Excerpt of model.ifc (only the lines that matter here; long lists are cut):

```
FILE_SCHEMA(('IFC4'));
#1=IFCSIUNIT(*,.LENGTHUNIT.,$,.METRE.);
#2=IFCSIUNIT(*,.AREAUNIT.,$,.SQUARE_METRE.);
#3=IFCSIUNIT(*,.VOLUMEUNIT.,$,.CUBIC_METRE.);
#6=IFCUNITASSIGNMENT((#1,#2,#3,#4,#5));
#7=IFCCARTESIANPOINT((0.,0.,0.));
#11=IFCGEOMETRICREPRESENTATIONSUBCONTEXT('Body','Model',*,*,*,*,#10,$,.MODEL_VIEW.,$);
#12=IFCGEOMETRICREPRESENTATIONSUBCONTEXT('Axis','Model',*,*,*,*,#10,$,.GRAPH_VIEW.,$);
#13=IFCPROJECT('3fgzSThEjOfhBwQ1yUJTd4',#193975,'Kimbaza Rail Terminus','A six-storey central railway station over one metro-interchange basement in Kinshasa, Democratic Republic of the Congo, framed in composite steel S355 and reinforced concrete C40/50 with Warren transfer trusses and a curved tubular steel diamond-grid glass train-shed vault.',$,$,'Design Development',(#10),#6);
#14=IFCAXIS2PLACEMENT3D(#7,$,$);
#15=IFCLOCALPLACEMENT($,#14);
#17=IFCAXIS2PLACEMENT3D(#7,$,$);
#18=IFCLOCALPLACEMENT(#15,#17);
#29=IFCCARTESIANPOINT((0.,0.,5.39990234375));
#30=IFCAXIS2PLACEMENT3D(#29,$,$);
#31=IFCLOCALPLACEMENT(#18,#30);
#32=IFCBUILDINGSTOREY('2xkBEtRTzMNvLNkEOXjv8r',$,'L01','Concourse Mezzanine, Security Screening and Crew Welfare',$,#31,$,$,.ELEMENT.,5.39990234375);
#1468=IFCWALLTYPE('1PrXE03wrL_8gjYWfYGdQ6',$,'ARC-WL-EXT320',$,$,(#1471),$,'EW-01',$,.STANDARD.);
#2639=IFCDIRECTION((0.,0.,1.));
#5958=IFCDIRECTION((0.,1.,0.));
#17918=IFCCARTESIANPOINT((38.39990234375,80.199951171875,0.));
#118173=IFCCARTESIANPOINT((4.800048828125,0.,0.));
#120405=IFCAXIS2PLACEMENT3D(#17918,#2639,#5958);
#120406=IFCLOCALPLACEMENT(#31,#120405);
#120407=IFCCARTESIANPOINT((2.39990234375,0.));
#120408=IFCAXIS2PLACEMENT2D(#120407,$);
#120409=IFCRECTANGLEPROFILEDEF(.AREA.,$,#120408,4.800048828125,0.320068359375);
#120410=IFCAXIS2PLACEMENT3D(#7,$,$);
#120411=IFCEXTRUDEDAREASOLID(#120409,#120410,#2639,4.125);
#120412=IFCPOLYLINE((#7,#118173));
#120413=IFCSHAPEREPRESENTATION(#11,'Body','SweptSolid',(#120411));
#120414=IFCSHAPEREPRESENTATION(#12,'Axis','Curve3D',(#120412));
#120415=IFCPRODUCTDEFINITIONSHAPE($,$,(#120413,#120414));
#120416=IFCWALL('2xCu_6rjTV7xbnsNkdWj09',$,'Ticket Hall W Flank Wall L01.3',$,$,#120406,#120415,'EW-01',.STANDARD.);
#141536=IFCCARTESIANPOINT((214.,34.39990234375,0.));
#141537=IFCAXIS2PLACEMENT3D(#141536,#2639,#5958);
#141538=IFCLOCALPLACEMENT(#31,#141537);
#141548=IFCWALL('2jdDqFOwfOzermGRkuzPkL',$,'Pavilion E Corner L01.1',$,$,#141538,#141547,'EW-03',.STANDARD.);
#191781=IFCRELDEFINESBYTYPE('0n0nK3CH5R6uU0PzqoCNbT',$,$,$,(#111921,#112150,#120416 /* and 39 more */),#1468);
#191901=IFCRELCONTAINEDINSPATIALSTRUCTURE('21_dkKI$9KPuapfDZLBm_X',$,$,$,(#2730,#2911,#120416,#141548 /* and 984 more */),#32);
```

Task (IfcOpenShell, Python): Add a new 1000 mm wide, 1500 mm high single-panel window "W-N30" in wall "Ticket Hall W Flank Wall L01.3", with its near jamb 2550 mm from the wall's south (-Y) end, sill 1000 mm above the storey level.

```python
import numpy as np
import ifcopenshell
import ifcopenshell.api.feature
import ifcopenshell.api.geometry
import ifcopenshell.api.root
import ifcopenshell.api.spatial
import ifcopenshell.geom
import ifcopenshell.util.element
import ifcopenshell.util.placement
import ifcopenshell.util.representation
import ifcopenshell.util.shape
import ifcopenshell.util.unit

model = ifcopenshell.open("model.ifc")
unit_scale = ifcopenshell.util.unit.calculate_unit_scale(model)
settings = ifcopenshell.geom.settings()


def volume(element):
    """Net volume in cubic metres, openings subtracted."""
    shape = ifcopenshell.geom.create_shape(settings, element)
    return ifcopenshell.util.shape.get_volume(shape.geometry)


wall = model.by_id(120416)
storey = ifcopenshell.util.element.get_container(wall, ifc_class="IfcBuildingStorey")
context = ifcopenshell.util.representation.get_context(model, "Model", "Body", "MODEL_VIEW")
before = volume(wall)

width, height, from_end, sill = 1, 1.5, 2.55, 1  # metres

# The wall runs along its own X axis, and the end named is its -X end.
wall_shape = ifcopenshell.geom.create_shape(settings, wall)
x, y, z = ifcopenshell.util.shape.get_vertices(wall_shape.geometry).T
start = x.min() + from_end
face, thickness = float(y.min()), float(y.max() - y.min())
wall_matrix = ifcopenshell.util.placement.get_local_placement(wall.ObjectPlacement)
level = ifcopenshell.util.placement.get_local_placement(storey.ObjectPlacement)[2, 3]


def in_wall(x, y):
    """Placement at x, y metres in the wall's axes, at sill height."""
    matrix = wall_matrix.copy()
    matrix[:, 3] = wall_matrix @ np.array([x / unit_scale, y / unit_scale, 0.0, 1.0])
    matrix[2, 3] = level + sill / unit_scale
    return matrix


# Opening: a box that overshoots both wall faces by 50 mm.
opening = ifcopenshell.api.root.create_entity(model, ifc_class="IfcOpeningElement", predefined_type="OPENING")
box = ifcopenshell.api.geometry.add_wall_representation(
    model, context=context, length=width, height=height, thickness=thickness + 0.1
)
ifcopenshell.api.geometry.assign_representation(model, product=opening, representation=box)
ifcopenshell.api.geometry.edit_object_placement(model, product=opening, matrix=in_wall(start, face - 0.05), is_si=False)
ifcopenshell.api.feature.add_feature(model, feature=opening, element=wall)

window = ifcopenshell.api.root.create_entity(model, ifc_class="IfcWindow", name="W-N30", predefined_type="WINDOW")
window.OverallWidth, window.OverallHeight = width / unit_scale, height / unit_scale
window.PartitioningType = "SINGLE_PANEL"
body = ifcopenshell.api.geometry.add_window_representation(
    model,
    context=context,
    overall_width=window.OverallWidth,
    overall_height=window.OverallHeight,
    partition_type="SINGLE_PANEL",
)
ifcopenshell.api.geometry.assign_representation(model, product=window, representation=body)
ifcopenshell.api.spatial.assign_container(model, products=[window], relating_structure=storey)
ifcopenshell.api.feature.add_filling(model, opening=opening, element=window)

# Centre the window in the wall's thickness.
ifcopenshell.api.geometry.edit_object_placement(model, product=window, matrix=in_wall(start, face), is_si=False)
window_shape = ifcopenshell.geom.create_shape(settings, window)
depth = ifcopenshell.util.shape.get_vertices(window_shape.geometry)[:, 1]
offset = face + thickness / 2 - (depth.min() + depth.max()) / 2
ifcopenshell.api.geometry.edit_object_placement(model, product=window, matrix=in_wall(start, offset), is_si=False)

after = volume(wall)

print(f"wall volume {before:.3f} -> {after:.3f} m3")

model.write("model_rev.ifc")
```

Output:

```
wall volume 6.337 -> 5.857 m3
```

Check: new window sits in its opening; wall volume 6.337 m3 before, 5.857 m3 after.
